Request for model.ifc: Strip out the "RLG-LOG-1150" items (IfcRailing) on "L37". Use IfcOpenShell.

First a look at what the model holds.

```python
import ifcopenshell
import ifcopenshell.util.element

model = ifcopenshell.open("model.ifc")
print(model.schema)
storey = next(s for s in model.by_type("IfcBuildingStorey") if s.Name == "L37")
railings = [e for e in ifcopenshell.util.element.get_decomposition(storey) if e.is_a("IfcRailing")]
seen = {}
for e in railings:
    element_type = ifcopenshell.util.element.get_type(e)
    name = element_type.Name if element_type not in (None, e) else None
    seen[name] = seen.get(name, 0) + 1
for name, count in sorted(seen.items(), key=str):
    print(count, "x", name)
```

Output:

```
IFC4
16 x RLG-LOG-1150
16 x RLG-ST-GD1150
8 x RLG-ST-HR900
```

```python
import ifcopenshell
import ifcopenshell.api.root
import ifcopenshell.util.element

model = ifcopenshell.open("model.ifc")

storey = next(s for s in model.by_type("IfcBuildingStorey") if s.Name == "L37")
railings = [e for e in ifcopenshell.util.element.get_decomposition(storey) if e.is_a("IfcRailing")]
targets = [e for e in railings if (t := ifcopenshell.util.element.get_type(e)) not in (None, e) and t.Name == "RLG-LOG-1150"]

for e in targets:
    ifcopenshell.api.root.remove_product(model, product=e)
print(len(targets), "removed")

model.write("model_rev.ifc")
```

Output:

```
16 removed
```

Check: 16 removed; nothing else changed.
